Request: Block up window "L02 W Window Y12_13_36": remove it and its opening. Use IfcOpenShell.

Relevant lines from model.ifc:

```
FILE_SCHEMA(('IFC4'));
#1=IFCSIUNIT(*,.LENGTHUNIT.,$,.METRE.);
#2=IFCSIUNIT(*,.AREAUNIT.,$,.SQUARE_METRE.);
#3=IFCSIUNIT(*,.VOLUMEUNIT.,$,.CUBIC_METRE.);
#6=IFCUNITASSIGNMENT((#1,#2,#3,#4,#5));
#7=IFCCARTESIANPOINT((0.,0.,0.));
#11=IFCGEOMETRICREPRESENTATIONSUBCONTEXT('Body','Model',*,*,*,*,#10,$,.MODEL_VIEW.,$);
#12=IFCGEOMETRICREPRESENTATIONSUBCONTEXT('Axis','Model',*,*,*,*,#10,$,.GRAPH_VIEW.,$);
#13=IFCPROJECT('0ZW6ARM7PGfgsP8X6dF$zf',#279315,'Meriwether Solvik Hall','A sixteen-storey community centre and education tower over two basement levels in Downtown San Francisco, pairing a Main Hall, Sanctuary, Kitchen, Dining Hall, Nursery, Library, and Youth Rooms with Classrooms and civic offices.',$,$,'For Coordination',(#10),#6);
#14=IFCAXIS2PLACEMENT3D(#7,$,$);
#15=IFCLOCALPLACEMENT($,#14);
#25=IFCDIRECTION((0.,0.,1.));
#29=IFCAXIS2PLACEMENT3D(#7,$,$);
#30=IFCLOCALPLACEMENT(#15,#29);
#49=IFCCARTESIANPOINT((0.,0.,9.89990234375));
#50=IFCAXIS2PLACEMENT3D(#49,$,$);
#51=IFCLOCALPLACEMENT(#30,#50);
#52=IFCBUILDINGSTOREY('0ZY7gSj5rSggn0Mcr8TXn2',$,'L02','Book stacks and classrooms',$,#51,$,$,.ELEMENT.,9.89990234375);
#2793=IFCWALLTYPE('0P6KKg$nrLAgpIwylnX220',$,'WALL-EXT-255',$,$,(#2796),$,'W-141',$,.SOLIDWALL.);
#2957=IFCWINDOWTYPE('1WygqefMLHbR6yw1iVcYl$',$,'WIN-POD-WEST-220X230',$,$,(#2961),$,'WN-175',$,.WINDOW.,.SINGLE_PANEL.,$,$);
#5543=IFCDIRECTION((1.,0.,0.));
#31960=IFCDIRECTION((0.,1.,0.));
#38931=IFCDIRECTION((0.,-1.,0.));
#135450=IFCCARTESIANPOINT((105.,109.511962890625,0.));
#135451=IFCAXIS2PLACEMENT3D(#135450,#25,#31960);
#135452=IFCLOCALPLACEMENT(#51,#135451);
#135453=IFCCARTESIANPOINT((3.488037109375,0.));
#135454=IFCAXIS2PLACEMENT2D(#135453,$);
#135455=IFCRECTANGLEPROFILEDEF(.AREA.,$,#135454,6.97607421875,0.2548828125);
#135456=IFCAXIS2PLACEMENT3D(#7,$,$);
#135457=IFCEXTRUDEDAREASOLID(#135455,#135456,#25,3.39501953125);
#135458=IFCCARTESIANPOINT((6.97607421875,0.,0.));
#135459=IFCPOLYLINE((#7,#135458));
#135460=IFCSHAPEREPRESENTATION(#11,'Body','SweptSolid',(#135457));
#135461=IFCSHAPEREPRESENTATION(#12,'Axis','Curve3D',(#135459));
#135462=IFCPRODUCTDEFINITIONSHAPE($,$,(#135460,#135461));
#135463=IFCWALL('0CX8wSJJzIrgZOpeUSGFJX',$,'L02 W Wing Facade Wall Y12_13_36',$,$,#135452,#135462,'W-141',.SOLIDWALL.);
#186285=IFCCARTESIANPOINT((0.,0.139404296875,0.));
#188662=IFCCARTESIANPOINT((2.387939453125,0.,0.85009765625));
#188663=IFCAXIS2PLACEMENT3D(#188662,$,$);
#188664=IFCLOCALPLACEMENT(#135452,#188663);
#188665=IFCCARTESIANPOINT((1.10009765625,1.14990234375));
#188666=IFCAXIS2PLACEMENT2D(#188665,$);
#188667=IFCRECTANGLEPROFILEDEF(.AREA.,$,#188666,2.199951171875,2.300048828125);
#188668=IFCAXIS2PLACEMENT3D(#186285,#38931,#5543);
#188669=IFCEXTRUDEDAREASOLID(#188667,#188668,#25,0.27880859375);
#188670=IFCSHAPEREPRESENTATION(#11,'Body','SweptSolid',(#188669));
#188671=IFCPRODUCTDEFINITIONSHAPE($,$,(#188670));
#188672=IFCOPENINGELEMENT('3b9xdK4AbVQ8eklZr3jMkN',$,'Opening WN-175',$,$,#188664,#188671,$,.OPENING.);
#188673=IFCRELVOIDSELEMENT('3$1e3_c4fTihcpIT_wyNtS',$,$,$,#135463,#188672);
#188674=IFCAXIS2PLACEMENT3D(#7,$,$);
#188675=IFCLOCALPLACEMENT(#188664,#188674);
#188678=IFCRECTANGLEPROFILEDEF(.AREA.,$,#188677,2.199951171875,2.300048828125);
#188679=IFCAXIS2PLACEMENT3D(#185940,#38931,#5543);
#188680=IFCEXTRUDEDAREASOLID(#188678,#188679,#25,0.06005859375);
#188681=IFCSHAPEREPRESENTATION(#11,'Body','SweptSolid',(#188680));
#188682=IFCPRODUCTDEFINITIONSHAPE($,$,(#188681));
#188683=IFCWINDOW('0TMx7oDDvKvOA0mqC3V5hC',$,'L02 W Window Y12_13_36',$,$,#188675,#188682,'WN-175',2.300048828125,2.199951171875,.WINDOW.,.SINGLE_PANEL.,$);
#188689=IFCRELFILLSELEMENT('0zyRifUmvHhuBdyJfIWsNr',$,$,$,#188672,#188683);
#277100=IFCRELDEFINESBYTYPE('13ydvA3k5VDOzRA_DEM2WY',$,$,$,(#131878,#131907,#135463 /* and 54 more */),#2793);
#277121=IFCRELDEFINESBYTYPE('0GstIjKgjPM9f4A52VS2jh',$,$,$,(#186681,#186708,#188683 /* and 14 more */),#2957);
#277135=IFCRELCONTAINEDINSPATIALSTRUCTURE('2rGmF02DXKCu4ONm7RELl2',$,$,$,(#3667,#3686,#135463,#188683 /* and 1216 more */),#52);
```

```python
import ifcopenshell
import ifcopenshell.api.feature
import ifcopenshell.api.root
import ifcopenshell.geom
import ifcopenshell.util.shape

model = ifcopenshell.open("model.ifc")
settings = ifcopenshell.geom.settings()


def volume(element):
    """Net volume in cubic metres, openings subtracted."""
    shape = ifcopenshell.geom.create_shape(settings, element)
    return ifcopenshell.util.shape.get_volume(shape.geometry)


window = model.by_guid("0TMx7oDDvKvOA0mqC3V5hC")
opening = window.FillsVoids[0].RelatingOpeningElement
wall = opening.VoidsElements[0].RelatingBuildingElement
before = volume(wall)

ifcopenshell.api.root.remove_product(model, product=window)
ifcopenshell.api.feature.remove_feature(model, feature=opening)

after = volume(wall)

print(f"wall volume {before:.3f} -> {after:.3f} m3")

model.write("model_updated.ifc")
```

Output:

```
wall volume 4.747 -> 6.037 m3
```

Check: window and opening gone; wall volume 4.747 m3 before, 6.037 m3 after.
